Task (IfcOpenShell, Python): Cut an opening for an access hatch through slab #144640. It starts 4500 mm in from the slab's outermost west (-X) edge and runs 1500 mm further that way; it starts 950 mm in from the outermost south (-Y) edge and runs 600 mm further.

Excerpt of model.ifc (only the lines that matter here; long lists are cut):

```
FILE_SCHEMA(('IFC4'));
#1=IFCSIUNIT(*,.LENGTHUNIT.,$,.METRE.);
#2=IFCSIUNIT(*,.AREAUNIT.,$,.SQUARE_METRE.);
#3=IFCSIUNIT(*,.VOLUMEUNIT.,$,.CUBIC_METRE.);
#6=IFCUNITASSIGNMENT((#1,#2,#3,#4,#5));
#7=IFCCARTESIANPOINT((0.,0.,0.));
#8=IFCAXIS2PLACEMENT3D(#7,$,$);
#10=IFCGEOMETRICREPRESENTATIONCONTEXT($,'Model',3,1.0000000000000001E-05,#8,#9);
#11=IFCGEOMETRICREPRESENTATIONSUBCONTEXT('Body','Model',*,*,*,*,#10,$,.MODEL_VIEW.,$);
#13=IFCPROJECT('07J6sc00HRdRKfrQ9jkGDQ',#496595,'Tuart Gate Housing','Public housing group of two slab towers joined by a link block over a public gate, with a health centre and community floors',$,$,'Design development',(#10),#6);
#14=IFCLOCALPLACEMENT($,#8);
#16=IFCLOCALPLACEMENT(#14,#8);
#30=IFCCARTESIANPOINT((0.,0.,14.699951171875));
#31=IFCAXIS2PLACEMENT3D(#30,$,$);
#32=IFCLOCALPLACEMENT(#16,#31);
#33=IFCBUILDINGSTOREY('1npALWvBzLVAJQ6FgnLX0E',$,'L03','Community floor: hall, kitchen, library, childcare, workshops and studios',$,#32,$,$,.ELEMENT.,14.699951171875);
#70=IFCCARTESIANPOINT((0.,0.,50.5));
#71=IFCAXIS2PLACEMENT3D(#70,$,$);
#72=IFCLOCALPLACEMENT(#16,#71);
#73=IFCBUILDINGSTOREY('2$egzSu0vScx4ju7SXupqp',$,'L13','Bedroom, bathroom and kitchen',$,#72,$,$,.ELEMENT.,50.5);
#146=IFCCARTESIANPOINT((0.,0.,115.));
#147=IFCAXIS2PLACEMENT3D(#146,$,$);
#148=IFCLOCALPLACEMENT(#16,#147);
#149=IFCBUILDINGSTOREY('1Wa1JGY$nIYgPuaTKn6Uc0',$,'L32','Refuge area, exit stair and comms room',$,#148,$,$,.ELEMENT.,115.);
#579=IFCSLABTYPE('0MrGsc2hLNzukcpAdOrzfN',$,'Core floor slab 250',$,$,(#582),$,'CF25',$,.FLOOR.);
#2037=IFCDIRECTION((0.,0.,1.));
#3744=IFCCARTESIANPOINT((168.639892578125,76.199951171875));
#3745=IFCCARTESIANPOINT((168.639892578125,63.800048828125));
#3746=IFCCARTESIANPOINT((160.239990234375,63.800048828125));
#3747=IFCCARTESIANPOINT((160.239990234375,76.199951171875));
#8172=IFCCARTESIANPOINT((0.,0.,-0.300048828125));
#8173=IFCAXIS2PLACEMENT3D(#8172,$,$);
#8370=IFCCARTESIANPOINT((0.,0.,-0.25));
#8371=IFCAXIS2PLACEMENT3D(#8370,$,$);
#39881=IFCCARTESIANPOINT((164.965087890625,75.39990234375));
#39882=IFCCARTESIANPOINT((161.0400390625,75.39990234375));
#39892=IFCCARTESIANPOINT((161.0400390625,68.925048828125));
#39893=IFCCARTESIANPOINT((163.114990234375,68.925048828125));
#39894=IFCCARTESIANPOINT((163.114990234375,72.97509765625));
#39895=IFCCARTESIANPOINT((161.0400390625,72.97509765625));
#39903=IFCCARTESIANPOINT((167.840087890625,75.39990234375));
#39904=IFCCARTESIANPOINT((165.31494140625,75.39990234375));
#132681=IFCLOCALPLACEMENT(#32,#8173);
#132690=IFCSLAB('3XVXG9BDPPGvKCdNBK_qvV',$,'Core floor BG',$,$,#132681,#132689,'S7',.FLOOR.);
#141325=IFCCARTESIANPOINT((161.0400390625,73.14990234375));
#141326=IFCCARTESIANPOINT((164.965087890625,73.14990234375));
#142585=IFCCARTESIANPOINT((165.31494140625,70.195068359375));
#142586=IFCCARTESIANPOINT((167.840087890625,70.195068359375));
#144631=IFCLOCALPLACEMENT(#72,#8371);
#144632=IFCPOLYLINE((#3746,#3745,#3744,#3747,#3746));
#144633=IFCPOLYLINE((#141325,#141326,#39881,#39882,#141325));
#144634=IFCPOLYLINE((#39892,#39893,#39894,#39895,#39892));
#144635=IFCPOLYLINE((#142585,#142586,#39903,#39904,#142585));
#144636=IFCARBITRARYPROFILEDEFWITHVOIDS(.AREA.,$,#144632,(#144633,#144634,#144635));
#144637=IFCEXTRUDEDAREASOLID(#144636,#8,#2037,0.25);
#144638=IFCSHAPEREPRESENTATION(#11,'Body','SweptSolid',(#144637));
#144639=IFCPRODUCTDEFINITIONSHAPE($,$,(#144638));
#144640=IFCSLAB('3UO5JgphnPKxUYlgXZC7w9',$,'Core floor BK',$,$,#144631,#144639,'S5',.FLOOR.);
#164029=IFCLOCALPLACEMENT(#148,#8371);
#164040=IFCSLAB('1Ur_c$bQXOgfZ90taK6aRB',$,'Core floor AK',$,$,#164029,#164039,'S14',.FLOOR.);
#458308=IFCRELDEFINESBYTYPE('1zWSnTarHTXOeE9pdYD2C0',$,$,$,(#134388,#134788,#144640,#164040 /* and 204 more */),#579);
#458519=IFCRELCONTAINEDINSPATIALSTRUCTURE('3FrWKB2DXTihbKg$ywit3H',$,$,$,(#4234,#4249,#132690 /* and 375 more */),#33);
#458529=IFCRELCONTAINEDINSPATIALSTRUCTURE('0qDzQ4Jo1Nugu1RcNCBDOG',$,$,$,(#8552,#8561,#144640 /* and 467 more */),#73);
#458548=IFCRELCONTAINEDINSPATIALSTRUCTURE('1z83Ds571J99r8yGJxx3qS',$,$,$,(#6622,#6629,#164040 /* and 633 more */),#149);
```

```python
import numpy as np
import ifcopenshell
import ifcopenshell.api.feature
import ifcopenshell.api.geometry
import ifcopenshell.api.root
import ifcopenshell.geom
import ifcopenshell.util.placement
import ifcopenshell.util.representation
import ifcopenshell.util.shape
import ifcopenshell.util.unit

model = ifcopenshell.open("model.ifc")
unit_scale = ifcopenshell.util.unit.calculate_unit_scale(model)
settings = ifcopenshell.geom.settings()


def volume(element):
    """Net volume in cubic metres, openings subtracted."""
    shape = ifcopenshell.geom.create_shape(settings, element)
    return ifcopenshell.util.shape.get_volume(shape.geometry)


slab = model.by_guid("3UO5JgphnPKxUYlgXZC7w9")
before = volume(slab)

# Extent in the slab's own axes, in metres. The edges named are its -X and -Y sides.
slab_shape = ifcopenshell.geom.create_shape(settings, slab)
vertices = ifcopenshell.util.shape.get_vertices(slab_shape.geometry)
x_min, y_min, bottom = vertices.min(axis=0)
top = vertices[:, 2].max()

opening = ifcopenshell.api.root.create_entity(model, ifc_class="IfcOpeningElement", name="Access hatch opening", predefined_type="OPENING")
context = ifcopenshell.util.representation.get_context(model, "Model", "Body", "MODEL_VIEW")
width, depth = 1.5, 0.6
outline = [(0.0, 0.0), (width, 0.0), (width, depth), (0.0, depth), (0.0, 0.0)]
# Overshoot both faces by 50 mm so the cut is clean.
shape = ifcopenshell.api.geometry.add_slab_representation(
    model, context=context, depth=top - bottom + 0.1, polyline=outline
)
ifcopenshell.api.geometry.assign_representation(model, product=opening, representation=shape)

matrix = ifcopenshell.util.placement.get_local_placement(slab.ObjectPlacement)
matrix[:, 3] = matrix @ np.append(np.array([x_min + 4.5, y_min + 0.95, bottom - 0.05]) / unit_scale, 1.0)
ifcopenshell.api.geometry.edit_object_placement(model, product=opening, matrix=matrix, is_si=False)
ifcopenshell.api.feature.add_feature(model, feature=opening, element=slab)

after = volume(slab)

print(f"slab volume {before:.3f} -> {after:.3f} m3")

model.write("model_edited.ifc")
```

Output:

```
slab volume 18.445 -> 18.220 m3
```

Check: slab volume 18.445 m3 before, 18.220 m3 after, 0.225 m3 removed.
